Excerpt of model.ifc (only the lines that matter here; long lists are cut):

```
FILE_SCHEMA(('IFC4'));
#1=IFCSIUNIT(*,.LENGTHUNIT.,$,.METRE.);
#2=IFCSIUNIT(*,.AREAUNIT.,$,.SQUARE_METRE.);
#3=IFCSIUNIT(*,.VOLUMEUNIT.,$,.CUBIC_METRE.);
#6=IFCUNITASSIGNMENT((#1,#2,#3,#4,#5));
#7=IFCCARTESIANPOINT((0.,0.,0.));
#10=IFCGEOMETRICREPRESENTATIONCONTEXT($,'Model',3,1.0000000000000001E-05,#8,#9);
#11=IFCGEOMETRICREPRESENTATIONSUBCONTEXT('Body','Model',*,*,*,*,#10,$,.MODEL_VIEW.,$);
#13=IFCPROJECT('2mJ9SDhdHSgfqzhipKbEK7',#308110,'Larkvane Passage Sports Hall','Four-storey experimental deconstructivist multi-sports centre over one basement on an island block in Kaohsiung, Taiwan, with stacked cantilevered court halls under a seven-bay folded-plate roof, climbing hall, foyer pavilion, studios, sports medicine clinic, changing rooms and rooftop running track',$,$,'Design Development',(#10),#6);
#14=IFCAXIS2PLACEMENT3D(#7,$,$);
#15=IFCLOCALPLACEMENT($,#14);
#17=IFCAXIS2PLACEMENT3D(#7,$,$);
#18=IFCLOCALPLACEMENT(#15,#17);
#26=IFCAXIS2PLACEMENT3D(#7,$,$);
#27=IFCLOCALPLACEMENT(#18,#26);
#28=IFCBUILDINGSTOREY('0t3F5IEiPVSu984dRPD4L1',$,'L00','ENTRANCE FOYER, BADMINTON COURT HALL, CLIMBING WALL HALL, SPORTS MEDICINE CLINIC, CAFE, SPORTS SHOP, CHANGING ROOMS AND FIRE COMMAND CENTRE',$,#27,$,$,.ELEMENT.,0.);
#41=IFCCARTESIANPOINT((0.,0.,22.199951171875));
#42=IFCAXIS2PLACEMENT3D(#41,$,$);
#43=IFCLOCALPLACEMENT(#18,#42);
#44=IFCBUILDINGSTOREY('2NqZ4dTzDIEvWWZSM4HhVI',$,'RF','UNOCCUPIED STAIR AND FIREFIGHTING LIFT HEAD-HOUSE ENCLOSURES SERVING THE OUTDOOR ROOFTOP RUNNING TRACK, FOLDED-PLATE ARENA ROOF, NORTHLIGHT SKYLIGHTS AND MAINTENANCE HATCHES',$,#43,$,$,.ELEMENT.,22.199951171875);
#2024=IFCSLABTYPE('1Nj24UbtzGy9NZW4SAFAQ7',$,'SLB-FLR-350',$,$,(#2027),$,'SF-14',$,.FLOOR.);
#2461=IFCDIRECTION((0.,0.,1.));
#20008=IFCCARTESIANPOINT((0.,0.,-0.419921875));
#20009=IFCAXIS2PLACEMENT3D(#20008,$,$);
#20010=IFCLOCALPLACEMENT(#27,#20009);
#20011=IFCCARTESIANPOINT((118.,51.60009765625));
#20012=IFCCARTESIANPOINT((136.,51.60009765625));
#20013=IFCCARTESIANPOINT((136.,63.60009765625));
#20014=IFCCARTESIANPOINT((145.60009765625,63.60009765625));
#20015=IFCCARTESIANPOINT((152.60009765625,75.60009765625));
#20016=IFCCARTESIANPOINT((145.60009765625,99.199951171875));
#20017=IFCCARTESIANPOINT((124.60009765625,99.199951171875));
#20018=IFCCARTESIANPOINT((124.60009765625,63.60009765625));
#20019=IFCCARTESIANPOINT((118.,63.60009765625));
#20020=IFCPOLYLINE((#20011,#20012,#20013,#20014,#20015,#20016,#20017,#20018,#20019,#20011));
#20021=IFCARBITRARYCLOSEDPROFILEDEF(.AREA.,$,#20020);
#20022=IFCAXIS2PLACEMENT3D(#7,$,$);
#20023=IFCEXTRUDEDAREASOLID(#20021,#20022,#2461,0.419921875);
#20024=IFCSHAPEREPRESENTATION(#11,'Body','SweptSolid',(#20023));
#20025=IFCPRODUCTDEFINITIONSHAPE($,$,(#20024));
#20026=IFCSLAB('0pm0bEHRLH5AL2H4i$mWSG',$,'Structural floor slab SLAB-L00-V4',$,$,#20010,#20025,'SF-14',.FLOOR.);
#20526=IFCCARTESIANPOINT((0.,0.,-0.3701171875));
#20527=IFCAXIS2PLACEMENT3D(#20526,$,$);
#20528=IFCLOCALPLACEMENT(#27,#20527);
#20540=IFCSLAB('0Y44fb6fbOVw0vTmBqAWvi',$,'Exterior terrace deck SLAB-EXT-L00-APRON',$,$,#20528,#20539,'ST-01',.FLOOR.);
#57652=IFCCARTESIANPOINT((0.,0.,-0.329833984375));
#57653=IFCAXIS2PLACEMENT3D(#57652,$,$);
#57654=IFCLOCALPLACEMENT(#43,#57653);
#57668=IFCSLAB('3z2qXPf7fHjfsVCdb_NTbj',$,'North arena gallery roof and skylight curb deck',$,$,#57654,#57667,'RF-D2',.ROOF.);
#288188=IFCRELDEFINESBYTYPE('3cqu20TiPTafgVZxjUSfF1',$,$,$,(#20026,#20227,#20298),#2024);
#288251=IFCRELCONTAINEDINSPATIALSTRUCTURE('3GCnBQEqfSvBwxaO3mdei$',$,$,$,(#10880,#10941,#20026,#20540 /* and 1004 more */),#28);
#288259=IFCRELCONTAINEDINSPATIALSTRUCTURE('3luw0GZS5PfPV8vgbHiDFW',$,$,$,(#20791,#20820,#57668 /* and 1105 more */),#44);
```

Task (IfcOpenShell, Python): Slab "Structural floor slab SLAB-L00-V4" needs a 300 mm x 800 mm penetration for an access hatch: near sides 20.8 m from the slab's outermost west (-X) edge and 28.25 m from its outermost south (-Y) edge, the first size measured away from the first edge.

```python
import numpy as np
import ifcopenshell
import ifcopenshell.api.feature
import ifcopenshell.api.geometry
import ifcopenshell.api.root
import ifcopenshell.geom
import ifcopenshell.util.placement
import ifcopenshell.util.representation
import ifcopenshell.util.shape
import ifcopenshell.util.unit

model = ifcopenshell.open("model.ifc")
unit_scale = ifcopenshell.util.unit.calculate_unit_scale(model)
settings = ifcopenshell.geom.settings()


def volume(element):
    """Net volume in cubic metres, openings subtracted."""
    shape = ifcopenshell.geom.create_shape(settings, element)
    return ifcopenshell.util.shape.get_volume(shape.geometry)


slab = model.by_guid("0pm0bEHRLH5AL2H4i$mWSG")
before = volume(slab)

# Extent in the slab's own axes, in metres. The edges named are its -X and -Y sides.
slab_shape = ifcopenshell.geom.create_shape(settings, slab)
vertices = ifcopenshell.util.shape.get_vertices(slab_shape.geometry)
x_min, y_min, bottom = vertices.min(axis=0)
top = vertices[:, 2].max()

opening = ifcopenshell.api.root.create_entity(model, ifc_class="IfcOpeningElement", name="Access hatch opening", predefined_type="OPENING")
context = ifcopenshell.util.representation.get_context(model, "Model", "Body", "MODEL_VIEW")
width, depth = 0.3, 0.8
outline = [(0.0, 0.0), (width, 0.0), (width, depth), (0.0, depth), (0.0, 0.0)]
# Overshoot both faces by 50 mm so the cut is clean.
shape = ifcopenshell.api.geometry.add_slab_representation(
    model, context=context, depth=top - bottom + 0.1, polyline=outline
)
ifcopenshell.api.geometry.assign_representation(model, product=opening, representation=shape)

matrix = ifcopenshell.util.placement.get_local_placement(slab.ObjectPlacement)
matrix[:, 3] = matrix @ np.append(np.array([x_min + 20.8, y_min + 28.25, bottom - 0.05]) / unit_scale, 1.0)
ifcopenshell.api.geometry.edit_object_placement(model, product=opening, matrix=matrix, is_si=False)
ifcopenshell.api.feature.add_feature(model, feature=opening, element=slab)

after = volume(slab)

print(f"slab volume {before:.3f} -> {after:.3f} m3")

model.write("model_v2.ifc")
```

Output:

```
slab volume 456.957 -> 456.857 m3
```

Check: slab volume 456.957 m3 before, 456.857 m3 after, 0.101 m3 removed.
